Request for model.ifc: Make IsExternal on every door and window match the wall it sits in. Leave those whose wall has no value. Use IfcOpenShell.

First a look at what the model holds.

```python
import ifcopenshell
import ifcopenshell.util.element

model = ifcopenshell.open("model.ifc")
print(model.schema)
seen = {}
for e in model.by_type("IfcDoor") + model.by_type("IfcWindow"):
    if not e.FillsVoids:
        continue
    host = e.FillsVoids[0].RelatingOpeningElement.VoidsElements[0].RelatingBuildingElement
    own = ifcopenshell.util.element.get_pset(e, f"Pset_{e.is_a()[3:].removesuffix('StandardCase')}Common", "IsExternal")
    wall = ifcopenshell.util.element.get_pset(host, "Pset_WallCommon", "IsExternal")
    seen[e.is_a(), own, wall] = seen.get((e.is_a(), own, wall), 0) + 1
for (cls, own, wall), count in sorted(seen.items(), key=str):
    print(count, cls, "IsExternal:", own, "| host wall:", wall)
```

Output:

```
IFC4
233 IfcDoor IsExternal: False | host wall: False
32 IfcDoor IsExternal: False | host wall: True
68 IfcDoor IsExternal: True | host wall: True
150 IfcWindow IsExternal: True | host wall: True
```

```python
import ifcopenshell
import ifcopenshell.api.pset
import ifcopenshell.util.element

model = ifcopenshell.open("model.ifc")

count = 0
for ifc_class, pset_name in (("IfcDoor", "Pset_DoorCommon"), ("IfcWindow", "Pset_WindowCommon")):
    for e in model.by_type(ifc_class):
        if not e.FillsVoids:
            continue
        host = e.FillsVoids[0].RelatingOpeningElement.VoidsElements[0].RelatingBuildingElement
        external = ifcopenshell.util.element.get_pset(host, "Pset_WallCommon", "IsExternal")
        if external is None or ifcopenshell.util.element.get_pset(e, pset_name, "IsExternal") == external:
            continue
        pset = ifcopenshell.api.pset.add_pset(model, product=e, name=pset_name)
        ifcopenshell.api.pset.edit_pset(model, pset=pset, properties={"IsExternal": external})
        count += 1

print(count, "updated")

model.write("model-out.ifc")
```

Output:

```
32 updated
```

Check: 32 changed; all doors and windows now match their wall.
